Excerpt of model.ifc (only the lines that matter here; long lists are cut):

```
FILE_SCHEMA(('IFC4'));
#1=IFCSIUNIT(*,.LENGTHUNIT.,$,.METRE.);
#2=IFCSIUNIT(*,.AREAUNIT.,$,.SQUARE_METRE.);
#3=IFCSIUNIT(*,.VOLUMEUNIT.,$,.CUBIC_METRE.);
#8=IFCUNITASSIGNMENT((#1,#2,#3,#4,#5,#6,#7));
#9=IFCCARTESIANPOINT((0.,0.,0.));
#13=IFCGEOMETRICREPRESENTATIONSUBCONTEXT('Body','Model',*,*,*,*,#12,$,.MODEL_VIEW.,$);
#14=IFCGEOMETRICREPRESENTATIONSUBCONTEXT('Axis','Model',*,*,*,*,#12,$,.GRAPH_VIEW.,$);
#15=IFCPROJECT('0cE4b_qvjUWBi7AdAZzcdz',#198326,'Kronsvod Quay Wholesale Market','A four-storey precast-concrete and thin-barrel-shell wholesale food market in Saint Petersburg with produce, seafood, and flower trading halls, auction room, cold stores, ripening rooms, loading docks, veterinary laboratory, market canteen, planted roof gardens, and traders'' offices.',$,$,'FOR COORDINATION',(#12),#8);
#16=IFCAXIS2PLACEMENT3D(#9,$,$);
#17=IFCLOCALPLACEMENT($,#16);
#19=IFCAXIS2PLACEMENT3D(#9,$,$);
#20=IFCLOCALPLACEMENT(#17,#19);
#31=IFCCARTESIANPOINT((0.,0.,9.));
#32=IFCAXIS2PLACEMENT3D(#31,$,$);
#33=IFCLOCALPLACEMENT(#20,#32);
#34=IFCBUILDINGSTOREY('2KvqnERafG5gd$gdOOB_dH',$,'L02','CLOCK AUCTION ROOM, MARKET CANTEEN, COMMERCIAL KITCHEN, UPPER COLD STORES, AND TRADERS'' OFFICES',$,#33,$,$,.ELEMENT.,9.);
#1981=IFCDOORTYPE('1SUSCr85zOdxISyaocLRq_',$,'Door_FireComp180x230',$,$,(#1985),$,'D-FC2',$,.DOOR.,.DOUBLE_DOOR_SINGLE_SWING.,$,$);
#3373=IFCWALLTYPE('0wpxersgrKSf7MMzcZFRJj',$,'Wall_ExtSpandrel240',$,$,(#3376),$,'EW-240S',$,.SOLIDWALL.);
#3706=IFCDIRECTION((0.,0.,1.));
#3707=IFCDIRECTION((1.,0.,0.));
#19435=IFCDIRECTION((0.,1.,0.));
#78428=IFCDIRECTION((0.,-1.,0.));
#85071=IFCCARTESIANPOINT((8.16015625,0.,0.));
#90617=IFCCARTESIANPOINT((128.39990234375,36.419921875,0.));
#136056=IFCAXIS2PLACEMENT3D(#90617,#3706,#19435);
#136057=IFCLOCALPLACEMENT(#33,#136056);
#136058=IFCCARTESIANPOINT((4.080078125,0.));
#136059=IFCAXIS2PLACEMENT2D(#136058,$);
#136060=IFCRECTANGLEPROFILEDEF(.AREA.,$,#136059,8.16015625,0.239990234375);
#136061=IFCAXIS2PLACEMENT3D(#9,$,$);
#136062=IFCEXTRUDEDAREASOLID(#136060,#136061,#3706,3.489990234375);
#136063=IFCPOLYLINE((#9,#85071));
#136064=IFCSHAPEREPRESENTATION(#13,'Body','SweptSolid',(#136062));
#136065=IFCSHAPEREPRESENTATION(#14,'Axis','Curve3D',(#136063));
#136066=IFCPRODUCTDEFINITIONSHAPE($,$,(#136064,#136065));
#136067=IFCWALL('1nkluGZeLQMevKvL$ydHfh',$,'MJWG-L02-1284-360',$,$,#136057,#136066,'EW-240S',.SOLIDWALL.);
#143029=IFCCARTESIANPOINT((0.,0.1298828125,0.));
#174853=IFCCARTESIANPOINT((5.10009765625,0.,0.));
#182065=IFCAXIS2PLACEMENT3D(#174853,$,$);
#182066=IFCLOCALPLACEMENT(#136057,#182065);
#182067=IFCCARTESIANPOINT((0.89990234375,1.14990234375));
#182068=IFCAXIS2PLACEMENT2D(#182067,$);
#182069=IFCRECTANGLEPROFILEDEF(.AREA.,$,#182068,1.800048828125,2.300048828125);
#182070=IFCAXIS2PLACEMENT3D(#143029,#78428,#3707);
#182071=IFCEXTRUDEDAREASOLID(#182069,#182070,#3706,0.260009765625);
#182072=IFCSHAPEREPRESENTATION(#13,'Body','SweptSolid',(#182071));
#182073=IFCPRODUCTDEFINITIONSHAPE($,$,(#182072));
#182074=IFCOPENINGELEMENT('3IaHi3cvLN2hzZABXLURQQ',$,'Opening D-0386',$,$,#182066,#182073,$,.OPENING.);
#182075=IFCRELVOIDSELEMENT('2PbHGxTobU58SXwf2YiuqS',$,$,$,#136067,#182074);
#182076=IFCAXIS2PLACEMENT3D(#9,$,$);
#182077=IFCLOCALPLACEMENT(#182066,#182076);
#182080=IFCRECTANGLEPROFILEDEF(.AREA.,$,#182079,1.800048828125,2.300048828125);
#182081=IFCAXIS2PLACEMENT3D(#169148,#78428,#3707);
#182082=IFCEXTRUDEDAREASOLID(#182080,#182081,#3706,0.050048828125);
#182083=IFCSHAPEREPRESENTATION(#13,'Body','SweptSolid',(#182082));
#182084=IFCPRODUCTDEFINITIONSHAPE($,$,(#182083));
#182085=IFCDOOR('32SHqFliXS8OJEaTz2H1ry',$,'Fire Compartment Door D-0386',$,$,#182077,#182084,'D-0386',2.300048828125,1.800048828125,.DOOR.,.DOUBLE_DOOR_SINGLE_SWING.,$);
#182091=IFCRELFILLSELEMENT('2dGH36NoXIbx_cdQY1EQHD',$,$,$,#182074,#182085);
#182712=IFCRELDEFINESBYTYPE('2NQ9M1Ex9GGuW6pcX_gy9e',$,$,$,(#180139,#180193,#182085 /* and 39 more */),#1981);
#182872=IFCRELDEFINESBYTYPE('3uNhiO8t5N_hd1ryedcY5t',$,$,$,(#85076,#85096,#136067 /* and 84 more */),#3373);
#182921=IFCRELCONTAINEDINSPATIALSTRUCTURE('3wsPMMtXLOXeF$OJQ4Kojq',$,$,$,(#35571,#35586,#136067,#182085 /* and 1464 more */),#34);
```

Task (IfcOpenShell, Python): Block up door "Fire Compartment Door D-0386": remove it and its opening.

```python
import ifcopenshell
import ifcopenshell.api.feature
import ifcopenshell.api.root
import ifcopenshell.geom
import ifcopenshell.util.shape

model = ifcopenshell.open("model.ifc")
settings = ifcopenshell.geom.settings()


def volume(element):
    """Net volume in cubic metres, openings subtracted."""
    shape = ifcopenshell.geom.create_shape(settings, element)
    return ifcopenshell.util.shape.get_volume(shape.geometry)


door = model.by_id(182085)
opening = door.FillsVoids[0].RelatingOpeningElement
wall = opening.VoidsElements[0].RelatingBuildingElement
before = volume(wall)

ifcopenshell.api.root.remove_product(model, product=door)
ifcopenshell.api.feature.remove_feature(model, feature=opening)

after = volume(wall)

print(f"wall volume {before:.3f} -> {after:.3f} m3")

model.write("model_updated.ifc")
```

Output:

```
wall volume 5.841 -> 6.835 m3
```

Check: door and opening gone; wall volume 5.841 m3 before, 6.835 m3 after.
